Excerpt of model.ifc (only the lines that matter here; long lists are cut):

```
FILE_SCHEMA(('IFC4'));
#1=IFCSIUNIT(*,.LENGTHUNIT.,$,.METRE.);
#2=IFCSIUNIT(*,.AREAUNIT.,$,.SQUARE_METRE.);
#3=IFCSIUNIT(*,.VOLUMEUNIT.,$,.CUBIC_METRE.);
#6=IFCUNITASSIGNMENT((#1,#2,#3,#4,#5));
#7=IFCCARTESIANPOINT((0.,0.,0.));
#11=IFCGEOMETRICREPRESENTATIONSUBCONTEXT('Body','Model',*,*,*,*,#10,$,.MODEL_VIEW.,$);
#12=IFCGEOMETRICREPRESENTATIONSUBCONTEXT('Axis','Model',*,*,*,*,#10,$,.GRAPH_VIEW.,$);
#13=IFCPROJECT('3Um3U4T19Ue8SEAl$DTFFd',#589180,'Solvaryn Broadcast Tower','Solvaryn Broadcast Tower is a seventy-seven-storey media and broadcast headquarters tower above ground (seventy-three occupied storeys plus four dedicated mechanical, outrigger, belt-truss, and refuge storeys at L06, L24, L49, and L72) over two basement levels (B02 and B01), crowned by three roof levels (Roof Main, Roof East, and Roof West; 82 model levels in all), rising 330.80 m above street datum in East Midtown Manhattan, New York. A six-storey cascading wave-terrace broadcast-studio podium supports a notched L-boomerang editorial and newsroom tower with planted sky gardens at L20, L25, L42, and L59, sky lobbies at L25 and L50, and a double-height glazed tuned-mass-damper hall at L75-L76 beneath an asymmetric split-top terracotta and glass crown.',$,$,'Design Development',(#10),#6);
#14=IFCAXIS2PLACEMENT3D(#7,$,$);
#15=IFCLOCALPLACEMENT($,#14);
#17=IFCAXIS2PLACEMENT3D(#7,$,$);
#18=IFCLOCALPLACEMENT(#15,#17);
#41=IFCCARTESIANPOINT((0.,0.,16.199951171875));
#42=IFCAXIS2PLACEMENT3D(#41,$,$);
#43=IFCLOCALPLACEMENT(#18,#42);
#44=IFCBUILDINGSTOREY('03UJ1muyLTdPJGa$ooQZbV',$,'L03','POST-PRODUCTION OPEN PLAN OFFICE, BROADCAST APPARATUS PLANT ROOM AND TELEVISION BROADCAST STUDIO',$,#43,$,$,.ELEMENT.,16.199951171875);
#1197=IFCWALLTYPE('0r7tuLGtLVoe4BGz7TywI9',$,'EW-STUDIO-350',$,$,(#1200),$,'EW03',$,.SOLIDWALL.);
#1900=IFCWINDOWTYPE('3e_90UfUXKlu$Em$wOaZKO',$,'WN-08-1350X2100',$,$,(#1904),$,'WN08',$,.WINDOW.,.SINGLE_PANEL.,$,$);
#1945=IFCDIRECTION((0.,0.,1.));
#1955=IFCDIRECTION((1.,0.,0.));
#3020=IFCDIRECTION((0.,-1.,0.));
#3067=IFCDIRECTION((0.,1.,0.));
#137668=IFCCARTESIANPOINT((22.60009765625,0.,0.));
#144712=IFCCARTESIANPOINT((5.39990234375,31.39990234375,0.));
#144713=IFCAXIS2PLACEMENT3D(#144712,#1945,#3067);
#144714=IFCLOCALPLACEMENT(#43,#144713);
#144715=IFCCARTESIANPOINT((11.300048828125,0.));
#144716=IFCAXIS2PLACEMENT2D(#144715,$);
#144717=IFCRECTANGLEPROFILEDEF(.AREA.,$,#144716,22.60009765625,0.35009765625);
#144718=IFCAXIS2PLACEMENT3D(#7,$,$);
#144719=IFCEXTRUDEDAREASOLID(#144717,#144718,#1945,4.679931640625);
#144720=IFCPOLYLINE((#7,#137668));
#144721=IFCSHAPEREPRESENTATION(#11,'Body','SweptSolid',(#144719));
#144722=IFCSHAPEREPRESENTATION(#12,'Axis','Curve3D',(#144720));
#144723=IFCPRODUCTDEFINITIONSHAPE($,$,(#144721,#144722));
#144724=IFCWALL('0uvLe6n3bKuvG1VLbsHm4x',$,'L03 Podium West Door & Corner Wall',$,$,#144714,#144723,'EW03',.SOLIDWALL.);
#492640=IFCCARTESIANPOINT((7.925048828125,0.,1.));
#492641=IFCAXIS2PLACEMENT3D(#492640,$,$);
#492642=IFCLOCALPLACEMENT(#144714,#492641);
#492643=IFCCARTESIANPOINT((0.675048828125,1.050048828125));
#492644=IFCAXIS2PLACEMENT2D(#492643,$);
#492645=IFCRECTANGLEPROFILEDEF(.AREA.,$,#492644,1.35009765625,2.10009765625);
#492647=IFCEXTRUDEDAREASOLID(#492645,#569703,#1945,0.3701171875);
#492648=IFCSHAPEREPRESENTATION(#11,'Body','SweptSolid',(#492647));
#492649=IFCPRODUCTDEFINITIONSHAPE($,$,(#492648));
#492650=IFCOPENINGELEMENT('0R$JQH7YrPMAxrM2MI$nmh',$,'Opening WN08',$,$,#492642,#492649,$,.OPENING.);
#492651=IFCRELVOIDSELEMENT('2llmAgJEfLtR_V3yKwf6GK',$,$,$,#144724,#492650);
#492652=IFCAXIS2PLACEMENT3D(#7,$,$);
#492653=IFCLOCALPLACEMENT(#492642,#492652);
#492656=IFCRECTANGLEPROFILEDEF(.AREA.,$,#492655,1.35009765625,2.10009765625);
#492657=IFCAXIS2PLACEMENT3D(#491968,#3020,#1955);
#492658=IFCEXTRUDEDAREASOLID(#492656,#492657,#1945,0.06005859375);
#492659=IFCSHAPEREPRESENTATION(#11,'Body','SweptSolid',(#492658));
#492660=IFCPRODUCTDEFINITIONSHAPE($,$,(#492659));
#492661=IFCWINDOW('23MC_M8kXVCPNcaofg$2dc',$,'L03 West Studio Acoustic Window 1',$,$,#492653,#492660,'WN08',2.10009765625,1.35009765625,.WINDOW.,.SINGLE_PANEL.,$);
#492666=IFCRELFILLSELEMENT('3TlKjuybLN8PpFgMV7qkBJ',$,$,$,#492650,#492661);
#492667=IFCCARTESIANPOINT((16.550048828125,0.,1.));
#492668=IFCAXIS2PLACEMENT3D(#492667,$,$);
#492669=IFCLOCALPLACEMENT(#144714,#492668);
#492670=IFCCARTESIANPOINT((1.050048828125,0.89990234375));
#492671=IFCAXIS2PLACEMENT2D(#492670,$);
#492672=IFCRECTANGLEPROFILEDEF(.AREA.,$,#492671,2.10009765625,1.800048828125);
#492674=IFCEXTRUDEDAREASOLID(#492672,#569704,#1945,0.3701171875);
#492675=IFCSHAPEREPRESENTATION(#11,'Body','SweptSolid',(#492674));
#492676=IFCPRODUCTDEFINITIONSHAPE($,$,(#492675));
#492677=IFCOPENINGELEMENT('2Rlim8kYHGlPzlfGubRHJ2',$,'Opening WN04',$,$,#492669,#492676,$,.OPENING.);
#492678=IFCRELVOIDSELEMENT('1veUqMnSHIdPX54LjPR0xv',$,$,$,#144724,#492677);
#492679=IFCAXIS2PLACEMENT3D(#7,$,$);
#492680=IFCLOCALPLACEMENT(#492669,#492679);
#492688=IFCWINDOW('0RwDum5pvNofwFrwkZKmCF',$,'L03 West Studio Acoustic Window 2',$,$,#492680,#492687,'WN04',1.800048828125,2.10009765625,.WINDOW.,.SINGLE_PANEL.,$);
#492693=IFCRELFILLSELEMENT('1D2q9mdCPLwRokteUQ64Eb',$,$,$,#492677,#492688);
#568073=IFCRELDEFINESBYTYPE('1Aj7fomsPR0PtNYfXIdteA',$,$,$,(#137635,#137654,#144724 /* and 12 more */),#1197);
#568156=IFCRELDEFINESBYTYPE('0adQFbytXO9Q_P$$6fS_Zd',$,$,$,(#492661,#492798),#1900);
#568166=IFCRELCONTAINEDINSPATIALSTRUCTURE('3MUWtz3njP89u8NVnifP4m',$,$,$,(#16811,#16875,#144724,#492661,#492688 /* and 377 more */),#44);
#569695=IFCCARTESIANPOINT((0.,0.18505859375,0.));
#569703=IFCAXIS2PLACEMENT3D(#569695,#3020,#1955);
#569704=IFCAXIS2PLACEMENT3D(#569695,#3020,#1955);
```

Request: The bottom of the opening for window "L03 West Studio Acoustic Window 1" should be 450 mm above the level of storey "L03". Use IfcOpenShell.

```python
import numpy as np
import ifcopenshell
import ifcopenshell.api.geometry
import ifcopenshell.geom
import ifcopenshell.util.element
import ifcopenshell.util.placement
import ifcopenshell.util.shape
import ifcopenshell.util.unit

model = ifcopenshell.open("model.ifc")
unit_scale = ifcopenshell.util.unit.calculate_unit_scale(model)

window = model.by_id(492661)
opening = window.FillsVoids[0].RelatingOpeningElement
storey = ifcopenshell.util.element.get_container(window, ifc_class="IfcBuildingStorey")
level = ifcopenshell.util.placement.get_local_placement(storey.ObjectPlacement)[2, 3]

# The opening's origin need not be at the sill, so measure its lowest point.
shape = ifcopenshell.geom.create_shape(ifcopenshell.geom.settings(), opening)
bottom = ifcopenshell.util.shape.get_shape_bottom_elevation(shape, shape.geometry) / unit_scale
dz = level + 0.45 - bottom

shift = np.array([0.0, 0.0, dz])
# The window is placed relative to its opening, so it follows when the opening moves.
matrix = ifcopenshell.util.placement.get_local_placement(opening.ObjectPlacement)
matrix[:3, 3] += shift
ifcopenshell.api.geometry.edit_object_placement(
    model, product=opening, matrix=matrix, is_si=False, should_transform_children=True
)

print(f"moved by {dz * unit_scale:+.3f} m")

model.write("model_rev.ifc")
```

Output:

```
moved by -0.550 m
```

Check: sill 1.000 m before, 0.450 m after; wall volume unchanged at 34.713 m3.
